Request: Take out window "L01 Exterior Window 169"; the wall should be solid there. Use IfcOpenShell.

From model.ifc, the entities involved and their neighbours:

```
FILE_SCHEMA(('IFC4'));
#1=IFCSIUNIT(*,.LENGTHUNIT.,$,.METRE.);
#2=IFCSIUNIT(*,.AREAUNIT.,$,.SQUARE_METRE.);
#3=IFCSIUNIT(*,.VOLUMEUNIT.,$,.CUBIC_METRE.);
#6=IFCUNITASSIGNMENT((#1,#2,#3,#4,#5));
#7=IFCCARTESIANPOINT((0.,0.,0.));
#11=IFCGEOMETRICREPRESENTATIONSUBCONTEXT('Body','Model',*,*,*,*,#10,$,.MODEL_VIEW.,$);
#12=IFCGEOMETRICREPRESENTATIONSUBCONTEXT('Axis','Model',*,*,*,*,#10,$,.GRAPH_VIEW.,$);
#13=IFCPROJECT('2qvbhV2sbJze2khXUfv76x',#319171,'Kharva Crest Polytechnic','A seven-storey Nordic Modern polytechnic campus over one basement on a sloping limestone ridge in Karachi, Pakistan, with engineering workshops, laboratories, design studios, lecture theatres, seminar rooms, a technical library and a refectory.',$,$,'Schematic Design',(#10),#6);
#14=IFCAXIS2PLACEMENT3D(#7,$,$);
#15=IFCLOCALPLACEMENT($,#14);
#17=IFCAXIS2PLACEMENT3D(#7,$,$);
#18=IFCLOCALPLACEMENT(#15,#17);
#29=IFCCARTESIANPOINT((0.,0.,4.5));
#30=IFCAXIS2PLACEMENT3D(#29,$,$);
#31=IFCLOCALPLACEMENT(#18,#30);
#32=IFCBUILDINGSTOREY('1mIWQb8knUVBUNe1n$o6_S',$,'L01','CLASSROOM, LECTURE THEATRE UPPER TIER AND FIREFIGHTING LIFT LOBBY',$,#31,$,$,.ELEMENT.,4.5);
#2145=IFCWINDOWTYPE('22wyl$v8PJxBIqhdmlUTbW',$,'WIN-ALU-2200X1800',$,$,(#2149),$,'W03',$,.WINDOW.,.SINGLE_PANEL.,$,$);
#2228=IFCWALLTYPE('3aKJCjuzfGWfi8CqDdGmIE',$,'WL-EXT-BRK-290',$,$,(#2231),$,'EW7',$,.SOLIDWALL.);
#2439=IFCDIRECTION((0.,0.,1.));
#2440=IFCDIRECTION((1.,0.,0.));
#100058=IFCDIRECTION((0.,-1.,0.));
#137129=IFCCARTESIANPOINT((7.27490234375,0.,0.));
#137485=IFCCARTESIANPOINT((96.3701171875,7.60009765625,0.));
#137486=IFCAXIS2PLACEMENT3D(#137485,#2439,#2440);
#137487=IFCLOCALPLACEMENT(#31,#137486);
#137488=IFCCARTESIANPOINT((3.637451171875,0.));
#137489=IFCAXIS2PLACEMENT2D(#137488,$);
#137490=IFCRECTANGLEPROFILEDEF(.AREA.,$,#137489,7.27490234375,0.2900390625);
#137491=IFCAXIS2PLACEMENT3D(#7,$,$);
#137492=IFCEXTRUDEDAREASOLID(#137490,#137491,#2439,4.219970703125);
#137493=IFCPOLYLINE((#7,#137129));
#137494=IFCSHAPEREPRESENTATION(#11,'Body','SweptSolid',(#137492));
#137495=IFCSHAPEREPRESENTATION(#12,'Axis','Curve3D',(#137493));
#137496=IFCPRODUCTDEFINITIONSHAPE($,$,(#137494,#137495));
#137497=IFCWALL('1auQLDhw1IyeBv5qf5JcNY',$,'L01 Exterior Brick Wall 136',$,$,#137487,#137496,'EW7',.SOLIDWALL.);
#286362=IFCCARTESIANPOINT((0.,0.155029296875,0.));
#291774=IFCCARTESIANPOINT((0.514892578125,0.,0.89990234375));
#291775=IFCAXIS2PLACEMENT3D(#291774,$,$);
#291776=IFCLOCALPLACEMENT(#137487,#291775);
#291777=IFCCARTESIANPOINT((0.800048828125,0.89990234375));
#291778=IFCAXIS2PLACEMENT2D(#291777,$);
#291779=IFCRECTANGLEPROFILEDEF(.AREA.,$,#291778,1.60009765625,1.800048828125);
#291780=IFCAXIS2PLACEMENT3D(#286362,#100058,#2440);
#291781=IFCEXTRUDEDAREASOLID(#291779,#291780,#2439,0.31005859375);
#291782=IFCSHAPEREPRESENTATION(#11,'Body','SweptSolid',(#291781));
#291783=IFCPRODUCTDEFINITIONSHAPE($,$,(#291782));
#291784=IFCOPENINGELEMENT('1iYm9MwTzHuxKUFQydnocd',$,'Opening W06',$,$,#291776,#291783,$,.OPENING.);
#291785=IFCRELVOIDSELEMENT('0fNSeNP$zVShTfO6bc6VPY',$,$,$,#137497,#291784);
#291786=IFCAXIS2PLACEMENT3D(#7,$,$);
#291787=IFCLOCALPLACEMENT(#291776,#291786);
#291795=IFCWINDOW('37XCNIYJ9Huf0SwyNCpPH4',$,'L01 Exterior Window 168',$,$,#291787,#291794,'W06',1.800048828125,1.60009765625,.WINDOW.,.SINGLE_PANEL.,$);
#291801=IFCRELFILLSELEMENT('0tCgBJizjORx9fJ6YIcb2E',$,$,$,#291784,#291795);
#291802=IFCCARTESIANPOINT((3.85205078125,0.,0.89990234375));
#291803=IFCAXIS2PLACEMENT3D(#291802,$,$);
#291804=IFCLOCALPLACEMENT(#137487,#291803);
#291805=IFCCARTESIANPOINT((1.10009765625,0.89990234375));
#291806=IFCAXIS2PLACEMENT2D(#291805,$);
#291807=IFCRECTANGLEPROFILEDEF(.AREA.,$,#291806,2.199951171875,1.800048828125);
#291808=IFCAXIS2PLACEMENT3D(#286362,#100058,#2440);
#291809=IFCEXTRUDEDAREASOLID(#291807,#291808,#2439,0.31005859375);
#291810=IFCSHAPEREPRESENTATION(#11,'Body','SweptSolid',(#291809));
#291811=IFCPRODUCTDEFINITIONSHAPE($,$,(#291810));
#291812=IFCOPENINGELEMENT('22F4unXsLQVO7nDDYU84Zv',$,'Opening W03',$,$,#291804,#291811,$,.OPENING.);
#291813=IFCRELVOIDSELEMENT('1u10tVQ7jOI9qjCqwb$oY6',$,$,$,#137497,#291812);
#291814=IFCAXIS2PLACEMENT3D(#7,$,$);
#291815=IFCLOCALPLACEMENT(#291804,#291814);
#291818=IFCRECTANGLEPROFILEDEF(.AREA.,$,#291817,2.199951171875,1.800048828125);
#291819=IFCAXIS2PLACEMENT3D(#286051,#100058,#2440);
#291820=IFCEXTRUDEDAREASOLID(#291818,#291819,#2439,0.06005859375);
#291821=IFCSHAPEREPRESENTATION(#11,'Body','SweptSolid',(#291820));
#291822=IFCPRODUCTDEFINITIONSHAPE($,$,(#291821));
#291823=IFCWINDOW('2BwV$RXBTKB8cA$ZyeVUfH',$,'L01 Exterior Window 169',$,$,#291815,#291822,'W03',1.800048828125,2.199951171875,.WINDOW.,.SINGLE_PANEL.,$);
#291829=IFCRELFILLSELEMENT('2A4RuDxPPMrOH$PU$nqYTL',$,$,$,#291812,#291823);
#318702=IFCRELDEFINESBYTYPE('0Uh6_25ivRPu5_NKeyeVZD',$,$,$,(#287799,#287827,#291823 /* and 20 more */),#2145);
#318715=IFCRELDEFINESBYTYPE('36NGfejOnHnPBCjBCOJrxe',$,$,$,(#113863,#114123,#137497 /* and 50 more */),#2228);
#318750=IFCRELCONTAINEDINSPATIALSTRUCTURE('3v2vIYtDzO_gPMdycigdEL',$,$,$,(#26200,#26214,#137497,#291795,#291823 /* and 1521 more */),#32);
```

```python
import ifcopenshell
import ifcopenshell.api.feature
import ifcopenshell.api.root
import ifcopenshell.geom
import ifcopenshell.util.shape

model = ifcopenshell.open("model.ifc")
settings = ifcopenshell.geom.settings()


def volume(element):
    """Net volume in cubic metres, openings subtracted."""
    shape = ifcopenshell.geom.create_shape(settings, element)
    return ifcopenshell.util.shape.get_volume(shape.geometry)


window = model.by_id(291823)
opening = window.FillsVoids[0].RelatingOpeningElement
wall = opening.VoidsElements[0].RelatingBuildingElement
before = volume(wall)

ifcopenshell.api.root.remove_product(model, product=window)
ifcopenshell.api.feature.remove_feature(model, feature=opening)

after = volume(wall)

print(f"wall volume {before:.3f} -> {after:.3f} m3")

model.write("model_updated.ifc")
```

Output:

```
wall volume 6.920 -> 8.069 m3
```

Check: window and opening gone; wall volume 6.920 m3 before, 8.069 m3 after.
